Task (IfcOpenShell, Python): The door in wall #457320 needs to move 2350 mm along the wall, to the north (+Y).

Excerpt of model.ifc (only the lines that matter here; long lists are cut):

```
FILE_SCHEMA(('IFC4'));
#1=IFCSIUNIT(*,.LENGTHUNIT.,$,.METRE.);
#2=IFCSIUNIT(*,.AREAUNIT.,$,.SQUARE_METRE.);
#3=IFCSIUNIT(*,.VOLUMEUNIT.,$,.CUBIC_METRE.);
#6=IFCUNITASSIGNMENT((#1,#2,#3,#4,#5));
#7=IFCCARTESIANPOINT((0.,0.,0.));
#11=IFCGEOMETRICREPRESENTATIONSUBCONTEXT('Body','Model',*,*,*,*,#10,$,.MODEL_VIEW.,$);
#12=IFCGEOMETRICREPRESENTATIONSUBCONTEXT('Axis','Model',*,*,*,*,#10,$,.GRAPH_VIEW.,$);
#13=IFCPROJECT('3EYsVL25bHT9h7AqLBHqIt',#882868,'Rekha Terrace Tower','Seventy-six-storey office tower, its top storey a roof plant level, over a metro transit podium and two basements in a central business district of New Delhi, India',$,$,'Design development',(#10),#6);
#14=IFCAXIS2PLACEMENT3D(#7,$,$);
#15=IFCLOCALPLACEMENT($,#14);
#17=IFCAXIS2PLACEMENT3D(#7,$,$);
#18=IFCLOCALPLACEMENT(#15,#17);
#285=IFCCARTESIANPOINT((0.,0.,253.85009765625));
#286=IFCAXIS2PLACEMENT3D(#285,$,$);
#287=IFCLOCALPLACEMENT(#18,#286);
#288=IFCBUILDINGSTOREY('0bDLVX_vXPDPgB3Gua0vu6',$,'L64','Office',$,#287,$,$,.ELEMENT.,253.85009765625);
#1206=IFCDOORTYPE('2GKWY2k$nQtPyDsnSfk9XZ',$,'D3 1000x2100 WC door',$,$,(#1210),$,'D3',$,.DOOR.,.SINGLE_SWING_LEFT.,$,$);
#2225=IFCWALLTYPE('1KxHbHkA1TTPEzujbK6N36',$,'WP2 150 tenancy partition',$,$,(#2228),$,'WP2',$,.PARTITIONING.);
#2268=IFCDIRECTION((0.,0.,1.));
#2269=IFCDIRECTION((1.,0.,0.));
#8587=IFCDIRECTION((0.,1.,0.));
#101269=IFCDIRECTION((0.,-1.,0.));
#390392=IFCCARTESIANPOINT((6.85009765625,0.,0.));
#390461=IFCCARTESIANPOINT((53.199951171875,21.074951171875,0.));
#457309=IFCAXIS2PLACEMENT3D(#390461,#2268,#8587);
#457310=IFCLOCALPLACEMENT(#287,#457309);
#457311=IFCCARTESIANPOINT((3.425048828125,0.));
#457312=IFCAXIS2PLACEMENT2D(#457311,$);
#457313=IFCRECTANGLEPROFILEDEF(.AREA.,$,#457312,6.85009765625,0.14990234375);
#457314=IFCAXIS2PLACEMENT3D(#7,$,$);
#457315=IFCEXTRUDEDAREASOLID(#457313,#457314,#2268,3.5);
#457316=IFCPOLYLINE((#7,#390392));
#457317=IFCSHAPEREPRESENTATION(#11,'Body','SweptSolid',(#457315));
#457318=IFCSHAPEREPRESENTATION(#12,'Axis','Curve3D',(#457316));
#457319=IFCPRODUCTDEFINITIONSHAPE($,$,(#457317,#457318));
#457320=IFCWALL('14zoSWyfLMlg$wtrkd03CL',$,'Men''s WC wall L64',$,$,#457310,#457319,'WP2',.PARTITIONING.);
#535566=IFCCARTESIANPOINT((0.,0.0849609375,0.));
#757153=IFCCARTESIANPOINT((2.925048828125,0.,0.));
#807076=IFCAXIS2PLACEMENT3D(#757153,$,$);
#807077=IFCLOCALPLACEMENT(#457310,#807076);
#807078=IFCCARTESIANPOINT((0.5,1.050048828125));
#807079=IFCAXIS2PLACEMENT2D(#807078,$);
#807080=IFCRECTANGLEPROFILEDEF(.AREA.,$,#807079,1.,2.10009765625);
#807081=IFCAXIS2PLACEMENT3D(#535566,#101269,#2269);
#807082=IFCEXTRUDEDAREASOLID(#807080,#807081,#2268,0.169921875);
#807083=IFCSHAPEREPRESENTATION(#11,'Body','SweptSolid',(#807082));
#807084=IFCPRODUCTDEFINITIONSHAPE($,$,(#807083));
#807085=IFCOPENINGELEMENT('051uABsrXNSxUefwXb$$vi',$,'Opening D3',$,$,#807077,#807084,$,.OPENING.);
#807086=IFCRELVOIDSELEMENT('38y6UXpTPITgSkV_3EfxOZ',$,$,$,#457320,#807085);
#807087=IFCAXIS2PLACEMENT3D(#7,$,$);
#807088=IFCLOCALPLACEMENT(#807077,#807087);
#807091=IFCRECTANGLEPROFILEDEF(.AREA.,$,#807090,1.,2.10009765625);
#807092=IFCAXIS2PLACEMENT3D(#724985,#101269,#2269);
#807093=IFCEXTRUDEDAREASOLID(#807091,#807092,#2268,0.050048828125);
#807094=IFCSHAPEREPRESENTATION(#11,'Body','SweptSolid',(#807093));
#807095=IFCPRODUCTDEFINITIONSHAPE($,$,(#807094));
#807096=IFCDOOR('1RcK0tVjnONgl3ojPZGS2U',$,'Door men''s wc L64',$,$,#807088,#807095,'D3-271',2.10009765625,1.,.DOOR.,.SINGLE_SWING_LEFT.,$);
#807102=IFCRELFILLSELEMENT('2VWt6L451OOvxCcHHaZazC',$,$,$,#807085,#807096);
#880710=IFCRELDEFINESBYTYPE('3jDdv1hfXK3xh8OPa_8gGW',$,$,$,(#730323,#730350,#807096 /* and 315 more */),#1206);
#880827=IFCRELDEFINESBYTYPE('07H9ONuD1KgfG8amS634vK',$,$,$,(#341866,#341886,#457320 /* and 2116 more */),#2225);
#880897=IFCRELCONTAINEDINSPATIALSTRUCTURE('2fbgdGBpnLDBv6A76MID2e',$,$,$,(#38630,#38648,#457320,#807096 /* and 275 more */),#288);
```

```python
import ifcopenshell
import ifcopenshell.api.geometry
import ifcopenshell.util.placement

model = ifcopenshell.open("model.ifc")

door = model.by_id(807096)
opening = door.FillsVoids[0].RelatingOpeningElement
wall = opening.VoidsElements[0].RelatingBuildingElement

wall_matrix = ifcopenshell.util.placement.get_local_placement(wall.ObjectPlacement)
shift = wall_matrix[:3, 0] * 2.35
before = ifcopenshell.util.placement.get_local_placement(door.ObjectPlacement)[:3, 3].copy()

# The door is placed relative to its opening, so it follows when the opening moves.
matrix = ifcopenshell.util.placement.get_local_placement(opening.ObjectPlacement)
matrix[:3, 3] += shift
ifcopenshell.api.geometry.edit_object_placement(
    model, product=opening, matrix=matrix, is_si=False, should_transform_children=True
)

after = ifcopenshell.util.placement.get_local_placement(door.ObjectPlacement)[:3, 3]
print("door moved by", (after - before).round(3) + 0.0)

model.write("model_rev.ifc")
```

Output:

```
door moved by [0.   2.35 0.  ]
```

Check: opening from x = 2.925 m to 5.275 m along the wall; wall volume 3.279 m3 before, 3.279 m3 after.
